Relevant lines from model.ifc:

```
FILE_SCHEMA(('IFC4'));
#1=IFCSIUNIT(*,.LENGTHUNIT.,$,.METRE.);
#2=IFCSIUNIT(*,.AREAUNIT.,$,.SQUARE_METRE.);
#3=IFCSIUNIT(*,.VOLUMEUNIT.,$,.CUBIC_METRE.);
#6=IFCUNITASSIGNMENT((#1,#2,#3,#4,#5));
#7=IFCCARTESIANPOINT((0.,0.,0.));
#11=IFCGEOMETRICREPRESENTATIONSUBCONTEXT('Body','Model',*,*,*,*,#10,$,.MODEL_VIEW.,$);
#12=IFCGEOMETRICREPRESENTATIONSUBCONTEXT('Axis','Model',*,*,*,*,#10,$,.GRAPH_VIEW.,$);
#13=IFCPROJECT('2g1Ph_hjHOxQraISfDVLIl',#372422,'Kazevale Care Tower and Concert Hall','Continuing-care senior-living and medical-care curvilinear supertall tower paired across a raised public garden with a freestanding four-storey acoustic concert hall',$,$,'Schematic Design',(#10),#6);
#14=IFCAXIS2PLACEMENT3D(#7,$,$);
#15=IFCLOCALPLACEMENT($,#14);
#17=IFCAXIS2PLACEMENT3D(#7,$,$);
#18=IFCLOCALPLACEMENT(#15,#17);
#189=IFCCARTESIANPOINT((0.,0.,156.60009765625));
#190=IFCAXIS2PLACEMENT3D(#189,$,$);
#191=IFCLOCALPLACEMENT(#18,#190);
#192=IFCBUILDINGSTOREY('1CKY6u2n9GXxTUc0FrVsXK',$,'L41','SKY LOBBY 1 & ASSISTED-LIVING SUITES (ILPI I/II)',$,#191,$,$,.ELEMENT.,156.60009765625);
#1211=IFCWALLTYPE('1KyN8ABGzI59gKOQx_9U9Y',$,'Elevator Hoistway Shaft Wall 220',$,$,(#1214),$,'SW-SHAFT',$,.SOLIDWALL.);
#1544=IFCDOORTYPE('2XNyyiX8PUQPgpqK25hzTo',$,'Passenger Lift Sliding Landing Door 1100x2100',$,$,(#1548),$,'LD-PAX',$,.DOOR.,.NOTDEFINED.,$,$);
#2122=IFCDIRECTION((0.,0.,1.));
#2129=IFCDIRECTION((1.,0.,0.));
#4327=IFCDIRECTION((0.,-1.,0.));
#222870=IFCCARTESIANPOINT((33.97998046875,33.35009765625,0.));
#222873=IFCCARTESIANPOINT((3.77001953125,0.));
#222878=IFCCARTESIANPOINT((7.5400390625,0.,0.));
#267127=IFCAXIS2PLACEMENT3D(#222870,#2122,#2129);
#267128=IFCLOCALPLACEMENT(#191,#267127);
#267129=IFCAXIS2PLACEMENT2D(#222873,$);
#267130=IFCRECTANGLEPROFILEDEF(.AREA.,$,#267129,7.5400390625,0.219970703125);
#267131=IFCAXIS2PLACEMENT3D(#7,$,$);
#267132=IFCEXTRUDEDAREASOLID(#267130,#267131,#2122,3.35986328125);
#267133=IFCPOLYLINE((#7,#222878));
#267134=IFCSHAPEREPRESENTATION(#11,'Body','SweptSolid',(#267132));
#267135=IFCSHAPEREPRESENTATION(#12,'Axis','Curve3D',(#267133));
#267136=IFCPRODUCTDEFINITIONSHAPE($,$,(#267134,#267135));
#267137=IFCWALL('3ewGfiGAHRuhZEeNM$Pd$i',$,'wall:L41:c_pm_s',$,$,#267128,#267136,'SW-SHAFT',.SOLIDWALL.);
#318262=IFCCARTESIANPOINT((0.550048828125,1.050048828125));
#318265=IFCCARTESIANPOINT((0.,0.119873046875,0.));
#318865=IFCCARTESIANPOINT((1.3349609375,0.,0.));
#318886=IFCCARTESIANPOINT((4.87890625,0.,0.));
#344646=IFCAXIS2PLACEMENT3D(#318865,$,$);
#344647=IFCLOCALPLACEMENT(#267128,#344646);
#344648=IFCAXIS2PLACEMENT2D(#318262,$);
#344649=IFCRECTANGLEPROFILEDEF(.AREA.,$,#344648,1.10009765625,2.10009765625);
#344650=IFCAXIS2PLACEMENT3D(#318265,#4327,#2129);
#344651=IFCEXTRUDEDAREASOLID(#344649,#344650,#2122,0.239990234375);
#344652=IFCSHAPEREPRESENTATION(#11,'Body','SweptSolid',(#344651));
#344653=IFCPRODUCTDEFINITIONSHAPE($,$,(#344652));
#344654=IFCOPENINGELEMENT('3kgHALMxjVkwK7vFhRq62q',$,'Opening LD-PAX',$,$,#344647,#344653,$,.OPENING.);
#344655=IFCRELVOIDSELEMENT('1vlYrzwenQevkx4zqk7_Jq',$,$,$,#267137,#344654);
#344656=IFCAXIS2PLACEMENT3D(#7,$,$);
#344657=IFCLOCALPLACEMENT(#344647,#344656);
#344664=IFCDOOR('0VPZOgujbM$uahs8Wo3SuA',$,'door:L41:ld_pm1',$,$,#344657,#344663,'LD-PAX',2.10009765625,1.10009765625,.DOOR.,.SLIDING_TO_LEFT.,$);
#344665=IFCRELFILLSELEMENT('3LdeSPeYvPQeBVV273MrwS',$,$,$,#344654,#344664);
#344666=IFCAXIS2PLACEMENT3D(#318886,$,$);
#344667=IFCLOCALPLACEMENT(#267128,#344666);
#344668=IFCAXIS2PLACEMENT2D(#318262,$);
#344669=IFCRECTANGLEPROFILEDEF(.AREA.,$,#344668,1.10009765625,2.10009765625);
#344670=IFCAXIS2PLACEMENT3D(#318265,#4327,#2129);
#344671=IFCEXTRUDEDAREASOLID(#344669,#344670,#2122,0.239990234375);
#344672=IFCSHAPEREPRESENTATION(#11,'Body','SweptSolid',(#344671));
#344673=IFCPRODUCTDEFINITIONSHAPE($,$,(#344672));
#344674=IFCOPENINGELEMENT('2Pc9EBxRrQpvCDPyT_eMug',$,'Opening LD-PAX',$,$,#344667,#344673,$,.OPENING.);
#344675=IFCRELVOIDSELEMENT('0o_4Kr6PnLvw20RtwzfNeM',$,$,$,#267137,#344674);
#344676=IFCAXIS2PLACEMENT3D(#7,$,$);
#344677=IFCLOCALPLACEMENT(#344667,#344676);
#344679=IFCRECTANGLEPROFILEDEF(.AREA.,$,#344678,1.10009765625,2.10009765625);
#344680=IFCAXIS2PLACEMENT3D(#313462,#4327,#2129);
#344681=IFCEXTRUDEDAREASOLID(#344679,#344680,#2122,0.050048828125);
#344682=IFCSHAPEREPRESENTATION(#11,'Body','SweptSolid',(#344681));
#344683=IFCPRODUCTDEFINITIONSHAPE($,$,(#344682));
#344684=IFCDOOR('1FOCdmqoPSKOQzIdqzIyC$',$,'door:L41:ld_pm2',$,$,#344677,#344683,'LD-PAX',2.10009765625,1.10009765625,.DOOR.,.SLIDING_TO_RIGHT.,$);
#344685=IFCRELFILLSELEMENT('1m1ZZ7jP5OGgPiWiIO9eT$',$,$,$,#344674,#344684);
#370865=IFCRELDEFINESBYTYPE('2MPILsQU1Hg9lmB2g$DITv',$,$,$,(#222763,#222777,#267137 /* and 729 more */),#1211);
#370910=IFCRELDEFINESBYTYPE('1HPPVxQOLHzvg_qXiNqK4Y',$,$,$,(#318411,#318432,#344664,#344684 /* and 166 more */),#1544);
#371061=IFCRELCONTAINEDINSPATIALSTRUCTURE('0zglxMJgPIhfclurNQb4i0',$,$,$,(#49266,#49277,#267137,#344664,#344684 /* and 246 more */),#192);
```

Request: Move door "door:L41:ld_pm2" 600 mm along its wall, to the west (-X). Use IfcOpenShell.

```python
import ifcopenshell
import ifcopenshell.api.geometry
import ifcopenshell.util.placement
import ifcopenshell.util.unit

model = ifcopenshell.open("model.ifc")
unit_scale = ifcopenshell.util.unit.calculate_unit_scale(model)

door = model.by_guid("1FOCdmqoPSKOQzIdqzIyC$")
opening = door.FillsVoids[0].RelatingOpeningElement
wall = opening.VoidsElements[0].RelatingBuildingElement

wall_matrix = ifcopenshell.util.placement.get_local_placement(wall.ObjectPlacement)
shift = wall_matrix[:3, 0] * -0.6 / unit_scale
before = ifcopenshell.util.placement.get_local_placement(door.ObjectPlacement)[:3, 3].copy()

# The door is placed relative to its opening, so it follows when the opening moves.
matrix = ifcopenshell.util.placement.get_local_placement(opening.ObjectPlacement)
matrix[:3, 3] += shift
ifcopenshell.api.geometry.edit_object_placement(
    model, product=opening, matrix=matrix, is_si=False, should_transform_children=True
)

after = ifcopenshell.util.placement.get_local_placement(door.ObjectPlacement)[:3, 3]
print("door moved by", (after - before).round(3) + 0.0)

model.write("model-out.ifc")
```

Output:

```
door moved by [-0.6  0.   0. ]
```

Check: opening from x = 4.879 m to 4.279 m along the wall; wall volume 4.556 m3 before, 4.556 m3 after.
